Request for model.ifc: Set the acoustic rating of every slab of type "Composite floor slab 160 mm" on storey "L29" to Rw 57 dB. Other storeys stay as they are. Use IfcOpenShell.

First a look at what the model holds.

```python
import ifcopenshell
import ifcopenshell.util.element

model = ifcopenshell.open("model.ifc")
print(model.schema)
storey = next(s for s in model.by_type("IfcBuildingStorey") if s.Name == "L29")
slabs = [e for e in ifcopenshell.util.element.get_decomposition(storey) if e.is_a("IfcSlab")]
seen = {}
for e in slabs:
    element_type = ifcopenshell.util.element.get_type(e)
    key = (element_type.Name if element_type != e and element_type else None, ifcopenshell.util.element.get_pset(e, "Pset_SlabCommon", "AcousticRating"))
    seen[key] = seen.get(key, 0) + 1
for (name, value), count in sorted(seen.items(), key=str):
    print(count, "x", name, "|", value)
```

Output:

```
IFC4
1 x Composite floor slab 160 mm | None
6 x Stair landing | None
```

```python
import ifcopenshell
import ifcopenshell.api.pset
import ifcopenshell.util.element

model = ifcopenshell.open("model.ifc")

storey = next(s for s in model.by_type("IfcBuildingStorey") if s.Name == "L29")
slabs = [e for e in ifcopenshell.util.element.get_decomposition(storey) if e.is_a("IfcSlab")]

count = 0
for e in slabs:
    element_type = ifcopenshell.util.element.get_type(e)
    if element_type in (None, e) or element_type.Name != "Composite floor slab 160 mm":
        continue
    found = ifcopenshell.util.element.get_pset(e, "Pset_SlabCommon", should_inherit=False)
    if found:
        pset = model.by_id(found["id"])
        if len(ifcopenshell.util.element.get_elements_by_pset(pset)) > 1:
            pset = ifcopenshell.api.pset.unshare_pset(model, products=[e], pset=pset)[0]
    else:
        pset = ifcopenshell.api.pset.add_pset(model, product=e, name="Pset_SlabCommon")
    ifcopenshell.api.pset.edit_pset(model, pset=pset, properties={"AcousticRating": "Rw 57 dB"})
    count += 1

print(count, "slabs updated")

model.write("model-out.ifc")
```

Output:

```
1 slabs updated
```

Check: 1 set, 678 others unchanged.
